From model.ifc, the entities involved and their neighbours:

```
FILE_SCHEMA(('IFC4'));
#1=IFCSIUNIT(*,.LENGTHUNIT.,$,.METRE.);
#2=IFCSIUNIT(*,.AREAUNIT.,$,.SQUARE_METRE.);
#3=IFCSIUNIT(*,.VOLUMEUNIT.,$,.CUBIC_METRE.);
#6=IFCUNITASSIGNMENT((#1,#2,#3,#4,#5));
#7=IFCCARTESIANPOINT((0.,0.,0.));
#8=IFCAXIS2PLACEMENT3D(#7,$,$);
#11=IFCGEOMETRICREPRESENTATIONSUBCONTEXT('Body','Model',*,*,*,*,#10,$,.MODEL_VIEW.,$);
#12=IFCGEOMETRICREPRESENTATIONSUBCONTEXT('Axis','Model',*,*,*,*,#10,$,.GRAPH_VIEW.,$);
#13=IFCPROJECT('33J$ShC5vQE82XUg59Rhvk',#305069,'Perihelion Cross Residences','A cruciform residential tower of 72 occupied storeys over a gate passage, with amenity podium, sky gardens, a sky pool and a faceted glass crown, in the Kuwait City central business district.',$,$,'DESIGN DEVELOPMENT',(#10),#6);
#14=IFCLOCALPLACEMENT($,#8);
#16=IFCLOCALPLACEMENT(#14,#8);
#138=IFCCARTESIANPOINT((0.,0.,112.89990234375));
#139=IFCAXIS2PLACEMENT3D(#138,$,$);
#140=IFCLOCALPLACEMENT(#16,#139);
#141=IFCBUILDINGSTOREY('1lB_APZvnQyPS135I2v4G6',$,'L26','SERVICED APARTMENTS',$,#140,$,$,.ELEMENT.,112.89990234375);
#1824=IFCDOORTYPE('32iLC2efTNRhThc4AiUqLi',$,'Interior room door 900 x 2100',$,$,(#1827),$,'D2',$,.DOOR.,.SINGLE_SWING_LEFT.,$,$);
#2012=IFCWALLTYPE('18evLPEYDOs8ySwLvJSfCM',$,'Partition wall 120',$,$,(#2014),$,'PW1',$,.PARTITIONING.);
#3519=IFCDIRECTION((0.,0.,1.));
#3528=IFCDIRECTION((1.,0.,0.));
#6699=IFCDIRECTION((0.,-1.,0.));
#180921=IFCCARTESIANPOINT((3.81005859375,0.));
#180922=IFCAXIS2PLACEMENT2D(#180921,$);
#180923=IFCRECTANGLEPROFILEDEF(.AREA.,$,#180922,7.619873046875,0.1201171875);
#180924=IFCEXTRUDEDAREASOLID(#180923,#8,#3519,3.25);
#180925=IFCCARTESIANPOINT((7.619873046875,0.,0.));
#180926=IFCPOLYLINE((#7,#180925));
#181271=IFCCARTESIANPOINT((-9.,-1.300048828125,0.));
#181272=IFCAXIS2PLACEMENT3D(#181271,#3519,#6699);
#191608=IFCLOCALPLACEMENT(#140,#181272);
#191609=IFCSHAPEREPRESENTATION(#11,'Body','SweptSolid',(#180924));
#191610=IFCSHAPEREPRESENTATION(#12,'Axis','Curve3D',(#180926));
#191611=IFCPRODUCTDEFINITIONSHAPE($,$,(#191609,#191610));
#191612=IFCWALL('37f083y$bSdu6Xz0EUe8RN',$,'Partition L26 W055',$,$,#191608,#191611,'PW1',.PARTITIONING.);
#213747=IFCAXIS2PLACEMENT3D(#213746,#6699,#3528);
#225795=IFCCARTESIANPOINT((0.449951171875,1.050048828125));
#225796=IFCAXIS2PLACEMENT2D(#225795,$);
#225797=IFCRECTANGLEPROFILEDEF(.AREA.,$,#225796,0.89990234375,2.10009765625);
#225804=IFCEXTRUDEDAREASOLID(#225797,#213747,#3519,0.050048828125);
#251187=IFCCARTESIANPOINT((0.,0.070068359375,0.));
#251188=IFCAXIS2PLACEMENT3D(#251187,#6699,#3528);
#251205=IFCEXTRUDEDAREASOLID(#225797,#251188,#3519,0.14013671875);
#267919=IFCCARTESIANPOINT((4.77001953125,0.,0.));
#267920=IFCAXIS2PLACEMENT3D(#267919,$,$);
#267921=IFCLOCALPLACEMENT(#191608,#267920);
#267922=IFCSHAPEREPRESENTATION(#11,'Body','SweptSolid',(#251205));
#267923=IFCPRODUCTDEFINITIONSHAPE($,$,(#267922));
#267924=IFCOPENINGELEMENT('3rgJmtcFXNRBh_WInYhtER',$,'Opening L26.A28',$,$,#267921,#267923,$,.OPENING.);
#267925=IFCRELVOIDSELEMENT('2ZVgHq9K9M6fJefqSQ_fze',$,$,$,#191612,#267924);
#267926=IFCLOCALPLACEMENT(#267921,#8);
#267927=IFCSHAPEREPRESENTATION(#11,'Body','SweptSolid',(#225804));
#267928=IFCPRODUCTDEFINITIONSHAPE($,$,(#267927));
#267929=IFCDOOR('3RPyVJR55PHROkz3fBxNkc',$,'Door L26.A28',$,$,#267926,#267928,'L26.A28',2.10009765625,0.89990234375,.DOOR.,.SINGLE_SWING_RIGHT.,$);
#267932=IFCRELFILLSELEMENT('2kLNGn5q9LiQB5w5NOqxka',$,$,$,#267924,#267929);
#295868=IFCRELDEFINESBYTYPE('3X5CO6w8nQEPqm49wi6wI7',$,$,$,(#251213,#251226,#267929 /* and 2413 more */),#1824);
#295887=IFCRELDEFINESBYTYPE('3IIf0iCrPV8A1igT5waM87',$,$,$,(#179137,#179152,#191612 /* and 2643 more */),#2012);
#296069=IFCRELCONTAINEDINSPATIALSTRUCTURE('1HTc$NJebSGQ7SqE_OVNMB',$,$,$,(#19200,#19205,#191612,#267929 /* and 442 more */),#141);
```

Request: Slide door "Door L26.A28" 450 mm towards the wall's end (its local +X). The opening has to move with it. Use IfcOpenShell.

```python
import ifcopenshell
import ifcopenshell.api.geometry
import ifcopenshell.util.placement
import ifcopenshell.util.unit

model = ifcopenshell.open("model.ifc")
unit_scale = ifcopenshell.util.unit.calculate_unit_scale(model)

door = model.by_id(267929)
opening = door.FillsVoids[0].RelatingOpeningElement
wall = opening.VoidsElements[0].RelatingBuildingElement

wall_matrix = ifcopenshell.util.placement.get_local_placement(wall.ObjectPlacement)
shift = wall_matrix[:3, 0] * 0.45 / unit_scale
before = ifcopenshell.util.placement.get_local_placement(door.ObjectPlacement)[:3, 3].copy()

# The door is placed relative to its opening, so it follows when the opening moves.
matrix = ifcopenshell.util.placement.get_local_placement(opening.ObjectPlacement)
matrix[:3, 3] += shift
ifcopenshell.api.geometry.edit_object_placement(
    model, product=opening, matrix=matrix, is_si=False, should_transform_children=True
)

after = ifcopenshell.util.placement.get_local_placement(door.ObjectPlacement)[:3, 3]
print("door moved by", (after - before).round(3) + 0.0)

model.write("model-out.ifc")
```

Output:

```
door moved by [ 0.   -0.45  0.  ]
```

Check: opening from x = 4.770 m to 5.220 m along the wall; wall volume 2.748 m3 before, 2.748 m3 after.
